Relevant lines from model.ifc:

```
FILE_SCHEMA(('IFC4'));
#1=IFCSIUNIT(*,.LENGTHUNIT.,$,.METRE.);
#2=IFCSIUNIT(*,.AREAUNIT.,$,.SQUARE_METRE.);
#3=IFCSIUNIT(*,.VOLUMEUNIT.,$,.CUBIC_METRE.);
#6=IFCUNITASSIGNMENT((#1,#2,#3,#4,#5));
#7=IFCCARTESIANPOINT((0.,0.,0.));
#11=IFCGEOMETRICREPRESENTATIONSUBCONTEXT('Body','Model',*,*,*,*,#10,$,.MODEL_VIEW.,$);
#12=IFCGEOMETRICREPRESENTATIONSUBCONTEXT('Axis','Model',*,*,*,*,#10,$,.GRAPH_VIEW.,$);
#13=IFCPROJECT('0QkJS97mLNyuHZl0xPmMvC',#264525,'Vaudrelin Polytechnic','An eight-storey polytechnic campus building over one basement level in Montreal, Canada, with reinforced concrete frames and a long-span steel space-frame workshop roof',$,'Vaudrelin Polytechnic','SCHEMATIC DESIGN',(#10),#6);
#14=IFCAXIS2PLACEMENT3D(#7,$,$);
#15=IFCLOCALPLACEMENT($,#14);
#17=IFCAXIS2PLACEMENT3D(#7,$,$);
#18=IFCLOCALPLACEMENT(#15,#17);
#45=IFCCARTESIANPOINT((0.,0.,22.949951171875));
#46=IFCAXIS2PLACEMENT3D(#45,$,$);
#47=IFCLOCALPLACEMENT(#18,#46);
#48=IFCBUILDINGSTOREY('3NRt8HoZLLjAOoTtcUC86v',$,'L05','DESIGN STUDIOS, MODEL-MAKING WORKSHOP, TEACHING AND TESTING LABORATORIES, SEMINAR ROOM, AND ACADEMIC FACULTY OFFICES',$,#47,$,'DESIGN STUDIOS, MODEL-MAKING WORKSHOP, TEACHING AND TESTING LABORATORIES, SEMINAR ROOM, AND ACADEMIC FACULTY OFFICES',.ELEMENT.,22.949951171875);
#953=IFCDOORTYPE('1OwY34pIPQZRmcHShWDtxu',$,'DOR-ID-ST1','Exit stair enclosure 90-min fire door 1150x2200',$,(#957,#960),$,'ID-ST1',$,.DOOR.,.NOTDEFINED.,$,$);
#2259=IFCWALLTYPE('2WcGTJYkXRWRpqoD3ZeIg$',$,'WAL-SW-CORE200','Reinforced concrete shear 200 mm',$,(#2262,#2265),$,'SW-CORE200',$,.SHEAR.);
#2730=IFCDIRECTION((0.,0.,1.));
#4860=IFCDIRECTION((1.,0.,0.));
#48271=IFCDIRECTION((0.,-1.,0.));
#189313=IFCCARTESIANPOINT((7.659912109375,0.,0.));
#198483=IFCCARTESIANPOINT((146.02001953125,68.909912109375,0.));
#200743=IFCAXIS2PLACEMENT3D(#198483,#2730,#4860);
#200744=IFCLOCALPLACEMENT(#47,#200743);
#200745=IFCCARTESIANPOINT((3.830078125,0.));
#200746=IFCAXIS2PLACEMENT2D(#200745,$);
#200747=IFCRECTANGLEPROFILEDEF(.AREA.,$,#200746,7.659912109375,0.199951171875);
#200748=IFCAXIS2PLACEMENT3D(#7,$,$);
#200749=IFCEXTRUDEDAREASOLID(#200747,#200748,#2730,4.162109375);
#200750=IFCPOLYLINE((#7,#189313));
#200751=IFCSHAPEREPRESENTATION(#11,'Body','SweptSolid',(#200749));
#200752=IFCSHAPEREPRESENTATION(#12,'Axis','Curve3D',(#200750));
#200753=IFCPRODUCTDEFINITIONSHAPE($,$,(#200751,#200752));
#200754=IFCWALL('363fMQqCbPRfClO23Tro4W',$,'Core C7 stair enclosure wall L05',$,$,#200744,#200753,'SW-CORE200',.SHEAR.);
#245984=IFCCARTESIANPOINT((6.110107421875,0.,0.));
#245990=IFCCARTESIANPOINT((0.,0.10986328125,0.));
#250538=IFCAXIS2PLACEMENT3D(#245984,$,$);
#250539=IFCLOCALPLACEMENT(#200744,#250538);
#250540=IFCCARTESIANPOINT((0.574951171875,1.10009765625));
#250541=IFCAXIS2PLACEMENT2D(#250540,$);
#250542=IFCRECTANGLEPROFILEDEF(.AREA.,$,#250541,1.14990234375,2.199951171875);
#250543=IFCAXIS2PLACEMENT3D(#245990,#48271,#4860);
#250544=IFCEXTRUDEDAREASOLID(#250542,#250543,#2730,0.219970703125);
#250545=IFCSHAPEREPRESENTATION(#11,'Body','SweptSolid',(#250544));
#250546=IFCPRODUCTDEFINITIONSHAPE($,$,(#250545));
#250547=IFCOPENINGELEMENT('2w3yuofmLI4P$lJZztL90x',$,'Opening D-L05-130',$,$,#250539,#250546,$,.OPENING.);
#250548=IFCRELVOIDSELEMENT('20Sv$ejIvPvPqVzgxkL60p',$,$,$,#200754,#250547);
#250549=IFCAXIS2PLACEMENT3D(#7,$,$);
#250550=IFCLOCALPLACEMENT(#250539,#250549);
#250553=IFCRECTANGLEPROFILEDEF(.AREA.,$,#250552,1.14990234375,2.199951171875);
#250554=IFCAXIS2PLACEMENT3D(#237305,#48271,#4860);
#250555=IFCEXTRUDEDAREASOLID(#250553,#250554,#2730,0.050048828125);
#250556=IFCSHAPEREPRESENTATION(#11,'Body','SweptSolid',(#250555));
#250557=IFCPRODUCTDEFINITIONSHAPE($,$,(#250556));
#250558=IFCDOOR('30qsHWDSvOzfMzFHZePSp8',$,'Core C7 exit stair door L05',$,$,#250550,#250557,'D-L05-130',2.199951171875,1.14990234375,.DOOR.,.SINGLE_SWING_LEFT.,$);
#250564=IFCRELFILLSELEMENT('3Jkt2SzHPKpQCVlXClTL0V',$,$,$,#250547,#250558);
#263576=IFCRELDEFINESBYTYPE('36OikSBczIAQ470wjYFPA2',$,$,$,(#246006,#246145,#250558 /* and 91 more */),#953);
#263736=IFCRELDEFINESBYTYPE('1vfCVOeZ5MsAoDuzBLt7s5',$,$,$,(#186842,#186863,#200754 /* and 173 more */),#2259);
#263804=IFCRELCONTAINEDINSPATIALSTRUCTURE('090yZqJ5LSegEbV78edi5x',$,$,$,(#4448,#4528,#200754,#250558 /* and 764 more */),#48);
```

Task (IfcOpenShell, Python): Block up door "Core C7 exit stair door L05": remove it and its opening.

```python
import ifcopenshell
import ifcopenshell.api.feature
import ifcopenshell.api.root
import ifcopenshell.geom
import ifcopenshell.util.shape

model = ifcopenshell.open("model.ifc")
settings = ifcopenshell.geom.settings()


def volume(element):
    """Net volume in cubic metres, openings subtracted."""
    shape = ifcopenshell.geom.create_shape(settings, element)
    return ifcopenshell.util.shape.get_volume(shape.geometry)


door = model.by_guid("30qsHWDSvOzfMzFHZePSp8")
opening = door.FillsVoids[0].RelatingOpeningElement
wall = opening.VoidsElements[0].RelatingBuildingElement
before = volume(wall)

ifcopenshell.api.root.remove_product(model, product=door)
ifcopenshell.api.feature.remove_feature(model, feature=opening)

after = volume(wall)

print(f"wall volume {before:.3f} -> {after:.3f} m3")

model.write("model_v2.ifc")
```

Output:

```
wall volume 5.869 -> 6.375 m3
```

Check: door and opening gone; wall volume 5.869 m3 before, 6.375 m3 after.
